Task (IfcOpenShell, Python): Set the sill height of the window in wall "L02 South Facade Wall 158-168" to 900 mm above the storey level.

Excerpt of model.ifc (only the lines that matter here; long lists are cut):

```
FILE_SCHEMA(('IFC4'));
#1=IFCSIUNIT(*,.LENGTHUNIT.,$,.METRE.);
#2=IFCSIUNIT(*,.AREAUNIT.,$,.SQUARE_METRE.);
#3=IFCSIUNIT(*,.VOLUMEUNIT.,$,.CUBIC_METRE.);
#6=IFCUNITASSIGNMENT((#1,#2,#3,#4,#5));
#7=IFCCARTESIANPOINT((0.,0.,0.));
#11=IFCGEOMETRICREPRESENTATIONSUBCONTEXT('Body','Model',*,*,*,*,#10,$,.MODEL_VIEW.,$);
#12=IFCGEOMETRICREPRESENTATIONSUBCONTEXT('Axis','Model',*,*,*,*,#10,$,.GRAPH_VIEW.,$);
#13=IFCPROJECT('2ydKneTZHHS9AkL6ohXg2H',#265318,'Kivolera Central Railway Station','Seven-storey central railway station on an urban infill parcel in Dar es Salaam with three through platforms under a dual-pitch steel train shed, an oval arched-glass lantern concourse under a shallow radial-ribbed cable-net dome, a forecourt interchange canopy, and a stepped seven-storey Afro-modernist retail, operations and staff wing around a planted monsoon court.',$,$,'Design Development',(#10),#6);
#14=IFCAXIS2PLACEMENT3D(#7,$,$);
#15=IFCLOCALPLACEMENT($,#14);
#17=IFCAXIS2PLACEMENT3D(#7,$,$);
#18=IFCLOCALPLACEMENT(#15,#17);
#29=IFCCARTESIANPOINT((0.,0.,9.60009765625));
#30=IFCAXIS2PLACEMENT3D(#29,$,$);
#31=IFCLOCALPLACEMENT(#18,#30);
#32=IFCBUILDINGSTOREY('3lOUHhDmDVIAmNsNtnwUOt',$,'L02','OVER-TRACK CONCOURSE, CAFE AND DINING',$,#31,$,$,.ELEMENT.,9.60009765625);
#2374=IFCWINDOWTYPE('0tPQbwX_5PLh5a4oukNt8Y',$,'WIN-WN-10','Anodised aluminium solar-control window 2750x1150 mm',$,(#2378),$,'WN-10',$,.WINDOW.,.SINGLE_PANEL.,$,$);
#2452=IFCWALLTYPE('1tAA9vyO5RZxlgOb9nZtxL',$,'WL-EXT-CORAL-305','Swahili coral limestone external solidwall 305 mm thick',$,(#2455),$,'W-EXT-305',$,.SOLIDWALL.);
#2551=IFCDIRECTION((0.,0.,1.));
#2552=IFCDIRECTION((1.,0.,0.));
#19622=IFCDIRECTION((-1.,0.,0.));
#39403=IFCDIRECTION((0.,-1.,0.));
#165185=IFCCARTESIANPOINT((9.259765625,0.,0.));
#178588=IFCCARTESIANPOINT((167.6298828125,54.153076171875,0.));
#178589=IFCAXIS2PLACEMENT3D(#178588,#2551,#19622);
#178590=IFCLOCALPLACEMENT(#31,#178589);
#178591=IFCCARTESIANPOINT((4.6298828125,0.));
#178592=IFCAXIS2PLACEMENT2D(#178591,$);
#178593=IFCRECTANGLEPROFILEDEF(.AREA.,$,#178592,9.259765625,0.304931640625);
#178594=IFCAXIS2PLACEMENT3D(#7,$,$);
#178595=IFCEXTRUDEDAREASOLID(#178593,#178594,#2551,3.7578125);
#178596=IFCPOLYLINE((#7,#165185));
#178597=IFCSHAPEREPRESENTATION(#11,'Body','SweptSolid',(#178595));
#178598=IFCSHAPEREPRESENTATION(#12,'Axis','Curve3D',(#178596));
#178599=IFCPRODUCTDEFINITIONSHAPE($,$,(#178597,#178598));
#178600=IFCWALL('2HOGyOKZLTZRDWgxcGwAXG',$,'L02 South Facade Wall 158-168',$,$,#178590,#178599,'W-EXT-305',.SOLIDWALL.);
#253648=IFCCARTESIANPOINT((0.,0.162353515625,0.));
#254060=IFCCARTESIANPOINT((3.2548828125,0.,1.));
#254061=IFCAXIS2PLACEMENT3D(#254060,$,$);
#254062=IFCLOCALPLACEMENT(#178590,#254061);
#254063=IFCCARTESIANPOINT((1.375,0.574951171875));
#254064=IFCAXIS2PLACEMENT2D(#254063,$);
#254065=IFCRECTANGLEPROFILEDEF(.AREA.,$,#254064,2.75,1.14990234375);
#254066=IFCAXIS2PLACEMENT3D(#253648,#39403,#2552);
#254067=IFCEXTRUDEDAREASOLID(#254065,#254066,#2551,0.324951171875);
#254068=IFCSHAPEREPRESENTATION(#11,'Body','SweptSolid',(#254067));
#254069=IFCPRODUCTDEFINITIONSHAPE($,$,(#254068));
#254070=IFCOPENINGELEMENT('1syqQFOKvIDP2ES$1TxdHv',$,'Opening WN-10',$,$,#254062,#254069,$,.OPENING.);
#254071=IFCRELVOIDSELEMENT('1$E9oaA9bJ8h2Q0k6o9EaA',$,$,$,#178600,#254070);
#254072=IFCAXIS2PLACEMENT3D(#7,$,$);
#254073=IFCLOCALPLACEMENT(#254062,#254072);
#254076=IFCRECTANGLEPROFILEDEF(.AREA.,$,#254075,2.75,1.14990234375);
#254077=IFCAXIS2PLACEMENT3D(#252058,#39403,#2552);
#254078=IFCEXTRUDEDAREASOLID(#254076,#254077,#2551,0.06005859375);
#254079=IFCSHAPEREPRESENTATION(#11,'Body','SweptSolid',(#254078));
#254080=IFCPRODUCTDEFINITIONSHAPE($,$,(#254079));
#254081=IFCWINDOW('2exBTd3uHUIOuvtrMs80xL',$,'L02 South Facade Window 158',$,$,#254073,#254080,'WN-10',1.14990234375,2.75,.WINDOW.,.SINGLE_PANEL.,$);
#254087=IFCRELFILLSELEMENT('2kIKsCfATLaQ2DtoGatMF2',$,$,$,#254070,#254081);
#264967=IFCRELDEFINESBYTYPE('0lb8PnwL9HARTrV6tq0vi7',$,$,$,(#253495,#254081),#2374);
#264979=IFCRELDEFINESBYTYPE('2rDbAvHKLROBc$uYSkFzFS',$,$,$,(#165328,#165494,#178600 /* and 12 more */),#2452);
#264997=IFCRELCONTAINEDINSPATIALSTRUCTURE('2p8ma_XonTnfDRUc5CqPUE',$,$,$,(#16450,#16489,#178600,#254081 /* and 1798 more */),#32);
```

```python
import numpy as np
import ifcopenshell
import ifcopenshell.api.geometry
import ifcopenshell.geom
import ifcopenshell.util.element
import ifcopenshell.util.placement
import ifcopenshell.util.shape
import ifcopenshell.util.unit

model = ifcopenshell.open("model.ifc")
unit_scale = ifcopenshell.util.unit.calculate_unit_scale(model)

window = model.by_guid("2exBTd3uHUIOuvtrMs80xL")
opening = window.FillsVoids[0].RelatingOpeningElement
storey = ifcopenshell.util.element.get_container(window, ifc_class="IfcBuildingStorey")
level = ifcopenshell.util.placement.get_local_placement(storey.ObjectPlacement)[2, 3]

# The opening's origin need not be at the sill, so measure its lowest point.
shape = ifcopenshell.geom.create_shape(ifcopenshell.geom.settings(), opening)
bottom = ifcopenshell.util.shape.get_shape_bottom_elevation(shape, shape.geometry) / unit_scale
dz = level + 0.9 / unit_scale - bottom

shift = np.array([0.0, 0.0, dz])
# The window is placed relative to its opening, so it follows when the opening moves.
matrix = ifcopenshell.util.placement.get_local_placement(opening.ObjectPlacement)
matrix[:3, 3] += shift
ifcopenshell.api.geometry.edit_object_placement(
    model, product=opening, matrix=matrix, is_si=False, should_transform_children=True
)

print(f"moved by {dz * unit_scale:+.3f} m")

model.write("model_edited.ifc")
```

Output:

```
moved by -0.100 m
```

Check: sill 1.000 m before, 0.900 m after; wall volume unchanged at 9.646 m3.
